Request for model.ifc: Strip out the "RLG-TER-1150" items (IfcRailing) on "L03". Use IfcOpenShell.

First a look at what the model holds.

```python
import ifcopenshell
import ifcopenshell.util.element

model = ifcopenshell.open("model.ifc")
print(model.schema)
storey = next(s for s in model.by_type("IfcBuildingStorey") if s.Name == "L03")
railings = [e for e in ifcopenshell.util.element.get_decomposition(storey) if e.is_a("IfcRailing")]
seen = {}
for e in railings:
    element_type = ifcopenshell.util.element.get_type(e)
    name = element_type.Name if element_type not in (None, e) else None
    seen[name] = seen.get(name, 0) + 1
for name, count in sorted(seen.items(), key=str):
    print(count, "x", name)
```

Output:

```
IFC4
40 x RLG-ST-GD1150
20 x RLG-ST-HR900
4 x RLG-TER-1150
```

```python
import ifcopenshell
import ifcopenshell.api.root
import ifcopenshell.util.element

model = ifcopenshell.open("model.ifc")

storey = next(s for s in model.by_type("IfcBuildingStorey") if s.Name == "L03")
railings = [e for e in ifcopenshell.util.element.get_decomposition(storey) if e.is_a("IfcRailing")]
targets = [e for e in railings if (t := ifcopenshell.util.element.get_type(e)) not in (None, e) and t.Name == "RLG-TER-1150"]

for e in targets:
    ifcopenshell.api.root.remove_product(model, product=e)
print(len(targets), "removed")

model.write("model_updated.ifc")
```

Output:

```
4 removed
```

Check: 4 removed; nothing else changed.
